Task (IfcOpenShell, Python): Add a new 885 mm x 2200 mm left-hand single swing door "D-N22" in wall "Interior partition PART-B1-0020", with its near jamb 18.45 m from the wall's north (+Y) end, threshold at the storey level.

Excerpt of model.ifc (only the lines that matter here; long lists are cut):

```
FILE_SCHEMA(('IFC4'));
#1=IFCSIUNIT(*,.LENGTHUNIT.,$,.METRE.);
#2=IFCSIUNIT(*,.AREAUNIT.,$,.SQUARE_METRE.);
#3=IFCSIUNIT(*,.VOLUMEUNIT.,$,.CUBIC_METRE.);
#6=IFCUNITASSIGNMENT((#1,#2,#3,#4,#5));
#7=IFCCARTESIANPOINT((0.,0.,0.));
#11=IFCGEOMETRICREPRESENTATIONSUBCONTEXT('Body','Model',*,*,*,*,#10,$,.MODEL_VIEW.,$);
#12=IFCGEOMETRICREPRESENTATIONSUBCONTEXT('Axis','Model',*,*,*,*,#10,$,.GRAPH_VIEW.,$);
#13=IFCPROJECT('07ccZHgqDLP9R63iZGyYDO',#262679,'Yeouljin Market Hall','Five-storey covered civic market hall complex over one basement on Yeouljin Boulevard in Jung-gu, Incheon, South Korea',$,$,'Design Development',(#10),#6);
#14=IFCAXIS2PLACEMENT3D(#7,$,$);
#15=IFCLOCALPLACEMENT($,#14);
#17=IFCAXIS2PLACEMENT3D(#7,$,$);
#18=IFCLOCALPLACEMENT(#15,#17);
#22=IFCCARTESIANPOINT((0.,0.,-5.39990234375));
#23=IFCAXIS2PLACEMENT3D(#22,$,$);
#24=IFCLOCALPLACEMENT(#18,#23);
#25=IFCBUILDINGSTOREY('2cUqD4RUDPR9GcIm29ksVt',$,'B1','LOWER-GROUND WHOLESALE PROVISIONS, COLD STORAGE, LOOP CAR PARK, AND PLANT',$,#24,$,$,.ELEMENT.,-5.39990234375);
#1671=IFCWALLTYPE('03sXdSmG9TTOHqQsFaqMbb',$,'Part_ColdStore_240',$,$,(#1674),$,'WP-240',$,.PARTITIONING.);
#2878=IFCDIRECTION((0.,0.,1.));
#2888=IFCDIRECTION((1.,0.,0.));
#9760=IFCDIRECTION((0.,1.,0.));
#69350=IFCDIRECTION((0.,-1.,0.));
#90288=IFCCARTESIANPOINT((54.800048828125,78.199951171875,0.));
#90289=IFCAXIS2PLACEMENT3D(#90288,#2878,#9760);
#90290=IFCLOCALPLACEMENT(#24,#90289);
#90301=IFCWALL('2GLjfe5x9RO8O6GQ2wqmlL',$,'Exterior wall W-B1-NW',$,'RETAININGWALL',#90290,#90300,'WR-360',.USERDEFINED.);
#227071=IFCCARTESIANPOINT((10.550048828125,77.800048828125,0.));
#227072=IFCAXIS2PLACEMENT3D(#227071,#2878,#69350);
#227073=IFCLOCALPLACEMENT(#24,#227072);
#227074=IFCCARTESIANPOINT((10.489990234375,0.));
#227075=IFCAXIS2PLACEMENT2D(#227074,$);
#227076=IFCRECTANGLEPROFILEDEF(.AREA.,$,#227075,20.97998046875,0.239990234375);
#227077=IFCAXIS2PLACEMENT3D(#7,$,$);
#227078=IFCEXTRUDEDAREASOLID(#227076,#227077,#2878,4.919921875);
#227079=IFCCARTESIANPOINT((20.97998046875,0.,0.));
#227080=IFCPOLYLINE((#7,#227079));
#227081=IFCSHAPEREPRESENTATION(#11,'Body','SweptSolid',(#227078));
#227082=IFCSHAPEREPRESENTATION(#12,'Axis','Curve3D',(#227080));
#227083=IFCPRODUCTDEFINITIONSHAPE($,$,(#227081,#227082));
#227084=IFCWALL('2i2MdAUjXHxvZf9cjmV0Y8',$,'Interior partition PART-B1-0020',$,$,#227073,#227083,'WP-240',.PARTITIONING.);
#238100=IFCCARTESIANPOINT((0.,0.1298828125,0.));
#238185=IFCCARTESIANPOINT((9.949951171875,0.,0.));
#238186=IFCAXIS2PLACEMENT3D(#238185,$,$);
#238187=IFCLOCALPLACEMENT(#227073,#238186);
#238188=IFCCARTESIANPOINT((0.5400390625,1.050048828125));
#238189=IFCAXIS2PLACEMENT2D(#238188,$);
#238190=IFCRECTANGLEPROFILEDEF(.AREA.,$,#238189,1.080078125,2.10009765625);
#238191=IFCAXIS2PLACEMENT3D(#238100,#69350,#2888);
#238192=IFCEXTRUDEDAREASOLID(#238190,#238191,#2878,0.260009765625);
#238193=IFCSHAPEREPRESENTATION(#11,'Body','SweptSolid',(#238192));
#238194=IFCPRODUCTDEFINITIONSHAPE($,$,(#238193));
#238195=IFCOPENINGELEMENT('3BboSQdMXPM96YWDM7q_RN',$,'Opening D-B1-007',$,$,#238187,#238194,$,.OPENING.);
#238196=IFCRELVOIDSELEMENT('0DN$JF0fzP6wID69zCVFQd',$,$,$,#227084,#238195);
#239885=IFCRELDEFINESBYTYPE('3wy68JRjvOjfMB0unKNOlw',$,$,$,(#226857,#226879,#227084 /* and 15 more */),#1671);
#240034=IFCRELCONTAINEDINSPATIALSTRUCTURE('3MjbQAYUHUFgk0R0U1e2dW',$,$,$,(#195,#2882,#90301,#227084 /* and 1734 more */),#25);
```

```python
import numpy as np
import ifcopenshell
import ifcopenshell.api.feature
import ifcopenshell.api.geometry
import ifcopenshell.api.root
import ifcopenshell.api.spatial
import ifcopenshell.geom
import ifcopenshell.util.element
import ifcopenshell.util.placement
import ifcopenshell.util.representation
import ifcopenshell.util.shape
import ifcopenshell.util.unit

model = ifcopenshell.open("model.ifc")
unit_scale = ifcopenshell.util.unit.calculate_unit_scale(model)
settings = ifcopenshell.geom.settings()


def volume(element):
    """Net volume in cubic metres, openings subtracted."""
    shape = ifcopenshell.geom.create_shape(settings, element)
    return ifcopenshell.util.shape.get_volume(shape.geometry)


wall = model.by_guid("2i2MdAUjXHxvZf9cjmV0Y8")
storey = ifcopenshell.util.element.get_container(wall, ifc_class="IfcBuildingStorey")
context = ifcopenshell.util.representation.get_context(model, "Model", "Body", "MODEL_VIEW")
before = volume(wall)

width, height, from_end, sill = 0.885, 2.2, 18.45, 0.0  # metres

# The wall runs along its own X axis, and the end named is its -X end.
wall_shape = ifcopenshell.geom.create_shape(settings, wall)
x, y, z = ifcopenshell.util.shape.get_vertices(wall_shape.geometry).T
start = x.min() + from_end
face, thickness = float(y.min()), float(y.max() - y.min())
wall_matrix = ifcopenshell.util.placement.get_local_placement(wall.ObjectPlacement)
level = ifcopenshell.util.placement.get_local_placement(storey.ObjectPlacement)[2, 3]


def in_wall(x, y):
    """Placement at x, y metres in the wall's axes, at sill height."""
    matrix = wall_matrix.copy()
    matrix[:, 3] = wall_matrix @ np.array([x / unit_scale, y / unit_scale, 0.0, 1.0])
    matrix[2, 3] = level + sill / unit_scale
    return matrix


# Opening: a box that overshoots both wall faces by 50 mm.
opening = ifcopenshell.api.root.create_entity(model, ifc_class="IfcOpeningElement", predefined_type="OPENING")
box = ifcopenshell.api.geometry.add_wall_representation(
    model, context=context, length=width, height=height, thickness=thickness + 0.1
)
ifcopenshell.api.geometry.assign_representation(model, product=opening, representation=box)
ifcopenshell.api.geometry.edit_object_placement(model, product=opening, matrix=in_wall(start, face - 0.05), is_si=False)
ifcopenshell.api.feature.add_feature(model, feature=opening, element=wall)

door = ifcopenshell.api.root.create_entity(model, ifc_class="IfcDoor", name="D-N22", predefined_type="DOOR")
door.OverallWidth, door.OverallHeight = width / unit_scale, height / unit_scale
door.OperationType = "SINGLE_SWING_LEFT"
body = ifcopenshell.api.geometry.add_door_representation(
    model,
    context=context,
    overall_width=door.OverallWidth,
    overall_height=door.OverallHeight,
    operation_type="SINGLE_SWING_LEFT",
    lining_properties={"LiningDepth": thickness / unit_scale, "ThresholdDepth": thickness / unit_scale},
)
ifcopenshell.api.geometry.assign_representation(model, product=door, representation=body)
ifcopenshell.api.spatial.assign_container(model, products=[door], relating_structure=storey)
ifcopenshell.api.feature.add_filling(model, opening=opening, element=door)

# The lining spans the wall, so the door starts at the wall face.
ifcopenshell.api.geometry.edit_object_placement(model, product=door, matrix=in_wall(start, face), is_si=False)

after = volume(wall)

print(f"wall volume {before:.3f} -> {after:.3f} m3")

model.write("model-out.ifc")
```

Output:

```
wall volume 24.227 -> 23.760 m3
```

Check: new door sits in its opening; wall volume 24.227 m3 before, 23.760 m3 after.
